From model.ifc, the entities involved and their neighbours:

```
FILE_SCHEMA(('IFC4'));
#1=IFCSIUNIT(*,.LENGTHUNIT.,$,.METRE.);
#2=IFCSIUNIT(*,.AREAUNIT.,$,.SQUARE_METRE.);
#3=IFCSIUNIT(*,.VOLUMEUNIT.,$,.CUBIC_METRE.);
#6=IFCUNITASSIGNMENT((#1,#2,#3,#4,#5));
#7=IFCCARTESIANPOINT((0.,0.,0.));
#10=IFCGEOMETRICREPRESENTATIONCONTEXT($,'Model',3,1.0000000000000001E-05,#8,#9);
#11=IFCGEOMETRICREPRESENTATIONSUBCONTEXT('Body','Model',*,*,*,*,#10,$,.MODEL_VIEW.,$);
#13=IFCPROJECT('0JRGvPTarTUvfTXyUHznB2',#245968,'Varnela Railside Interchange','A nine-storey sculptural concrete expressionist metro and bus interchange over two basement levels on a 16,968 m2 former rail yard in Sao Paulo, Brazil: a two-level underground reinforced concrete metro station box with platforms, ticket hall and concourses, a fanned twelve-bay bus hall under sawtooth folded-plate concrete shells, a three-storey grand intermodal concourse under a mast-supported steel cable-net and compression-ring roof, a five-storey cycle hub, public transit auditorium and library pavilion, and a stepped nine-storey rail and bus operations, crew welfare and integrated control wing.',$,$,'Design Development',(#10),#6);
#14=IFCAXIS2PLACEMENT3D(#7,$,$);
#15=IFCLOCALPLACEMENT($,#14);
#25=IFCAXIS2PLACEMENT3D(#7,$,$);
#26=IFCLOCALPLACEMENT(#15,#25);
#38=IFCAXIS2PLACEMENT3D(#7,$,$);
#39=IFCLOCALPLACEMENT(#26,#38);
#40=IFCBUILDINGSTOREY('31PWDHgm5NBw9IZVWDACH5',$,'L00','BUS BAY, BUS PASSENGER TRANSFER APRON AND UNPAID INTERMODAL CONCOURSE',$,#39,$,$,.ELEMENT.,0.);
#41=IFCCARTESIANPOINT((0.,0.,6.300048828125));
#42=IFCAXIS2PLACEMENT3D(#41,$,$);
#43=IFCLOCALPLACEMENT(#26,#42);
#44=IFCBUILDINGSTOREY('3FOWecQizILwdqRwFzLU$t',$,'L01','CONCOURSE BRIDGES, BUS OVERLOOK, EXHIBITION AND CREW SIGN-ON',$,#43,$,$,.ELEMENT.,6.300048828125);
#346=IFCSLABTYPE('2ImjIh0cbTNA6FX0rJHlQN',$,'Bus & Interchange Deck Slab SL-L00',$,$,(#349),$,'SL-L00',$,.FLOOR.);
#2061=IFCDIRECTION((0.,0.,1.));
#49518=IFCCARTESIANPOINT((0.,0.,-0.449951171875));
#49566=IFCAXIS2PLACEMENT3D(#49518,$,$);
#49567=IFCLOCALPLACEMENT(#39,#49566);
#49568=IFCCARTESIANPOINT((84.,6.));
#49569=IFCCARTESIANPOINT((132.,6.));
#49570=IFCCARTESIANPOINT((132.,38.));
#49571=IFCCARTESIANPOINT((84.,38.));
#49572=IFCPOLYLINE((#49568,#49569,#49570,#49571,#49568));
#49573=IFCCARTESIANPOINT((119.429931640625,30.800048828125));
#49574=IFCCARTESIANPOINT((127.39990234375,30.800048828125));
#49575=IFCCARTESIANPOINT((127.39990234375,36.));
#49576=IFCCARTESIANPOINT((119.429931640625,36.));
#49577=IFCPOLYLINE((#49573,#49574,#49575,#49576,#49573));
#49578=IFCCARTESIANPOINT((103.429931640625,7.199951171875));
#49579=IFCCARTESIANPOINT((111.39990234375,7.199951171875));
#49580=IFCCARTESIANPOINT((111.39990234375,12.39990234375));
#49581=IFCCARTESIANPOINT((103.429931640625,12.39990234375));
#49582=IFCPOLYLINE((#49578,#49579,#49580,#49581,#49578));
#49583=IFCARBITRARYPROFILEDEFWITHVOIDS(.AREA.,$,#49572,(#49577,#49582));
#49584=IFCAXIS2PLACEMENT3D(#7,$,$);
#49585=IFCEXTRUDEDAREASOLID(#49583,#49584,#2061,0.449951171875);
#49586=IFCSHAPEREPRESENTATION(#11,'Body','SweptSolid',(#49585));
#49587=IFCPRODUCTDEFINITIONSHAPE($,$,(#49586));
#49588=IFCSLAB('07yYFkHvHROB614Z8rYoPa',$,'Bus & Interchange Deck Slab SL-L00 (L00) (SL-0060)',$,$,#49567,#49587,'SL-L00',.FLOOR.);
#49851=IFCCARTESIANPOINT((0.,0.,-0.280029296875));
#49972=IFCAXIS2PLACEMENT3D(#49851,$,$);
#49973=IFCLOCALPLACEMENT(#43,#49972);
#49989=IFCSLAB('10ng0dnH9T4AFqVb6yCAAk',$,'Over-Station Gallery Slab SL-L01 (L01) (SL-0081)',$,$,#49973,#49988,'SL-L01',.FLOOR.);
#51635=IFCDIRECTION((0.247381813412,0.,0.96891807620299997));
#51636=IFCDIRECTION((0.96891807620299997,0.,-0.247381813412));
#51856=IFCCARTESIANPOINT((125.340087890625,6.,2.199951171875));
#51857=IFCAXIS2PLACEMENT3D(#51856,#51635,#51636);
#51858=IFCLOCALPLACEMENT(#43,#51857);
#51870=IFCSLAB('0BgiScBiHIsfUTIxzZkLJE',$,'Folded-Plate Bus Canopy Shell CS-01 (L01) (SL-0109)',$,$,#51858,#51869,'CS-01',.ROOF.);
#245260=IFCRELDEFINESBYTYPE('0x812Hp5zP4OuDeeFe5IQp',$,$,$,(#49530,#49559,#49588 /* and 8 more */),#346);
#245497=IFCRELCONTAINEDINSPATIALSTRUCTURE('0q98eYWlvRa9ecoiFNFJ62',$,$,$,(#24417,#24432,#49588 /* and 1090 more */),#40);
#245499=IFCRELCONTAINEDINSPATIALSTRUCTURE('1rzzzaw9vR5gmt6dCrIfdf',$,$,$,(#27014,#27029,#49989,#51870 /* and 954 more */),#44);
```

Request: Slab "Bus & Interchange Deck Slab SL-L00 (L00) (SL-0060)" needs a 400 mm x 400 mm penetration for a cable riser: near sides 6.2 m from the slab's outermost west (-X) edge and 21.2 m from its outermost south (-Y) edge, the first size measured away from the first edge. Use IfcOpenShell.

```python
import numpy as np
import ifcopenshell
import ifcopenshell.api.feature
import ifcopenshell.api.geometry
import ifcopenshell.api.root
import ifcopenshell.geom
import ifcopenshell.util.placement
import ifcopenshell.util.representation
import ifcopenshell.util.shape
import ifcopenshell.util.unit

model = ifcopenshell.open("model.ifc")
unit_scale = ifcopenshell.util.unit.calculate_unit_scale(model)
settings = ifcopenshell.geom.settings()


def volume(element):
    """Net volume in cubic metres, openings subtracted."""
    shape = ifcopenshell.geom.create_shape(settings, element)
    return ifcopenshell.util.shape.get_volume(shape.geometry)


slab = model.by_guid("07yYFkHvHROB614Z8rYoPa")
before = volume(slab)

# Extent in the slab's own axes, in metres. The edges named are its -X and -Y sides.
slab_shape = ifcopenshell.geom.create_shape(settings, slab)
vertices = ifcopenshell.util.shape.get_vertices(slab_shape.geometry)
x_min, y_min, bottom = vertices.min(axis=0)
top = vertices[:, 2].max()

opening = ifcopenshell.api.root.create_entity(model, ifc_class="IfcOpeningElement", name="Cable riser opening", predefined_type="OPENING")
context = ifcopenshell.util.representation.get_context(model, "Model", "Body", "MODEL_VIEW")
width, depth = 0.4, 0.4
outline = [(0.0, 0.0), (width, 0.0), (width, depth), (0.0, depth), (0.0, 0.0)]
# Overshoot both faces by 50 mm so the cut is clean.
shape = ifcopenshell.api.geometry.add_slab_representation(
    model, context=context, depth=top - bottom + 0.1, polyline=outline
)
ifcopenshell.api.geometry.assign_representation(model, product=opening, representation=shape)

matrix = ifcopenshell.util.placement.get_local_placement(slab.ObjectPlacement)
matrix[:, 3] = matrix @ np.append(np.array([x_min + 6.2, y_min + 21.2, bottom - 0.05]) / unit_scale, 1.0)
ifcopenshell.api.geometry.edit_object_placement(model, product=opening, matrix=matrix, is_si=False)
ifcopenshell.api.feature.add_feature(model, feature=opening, element=slab)

after = volume(slab)

print(f"slab volume {before:.3f} -> {after:.3f} m3")

model.write("model_v2.ifc")
```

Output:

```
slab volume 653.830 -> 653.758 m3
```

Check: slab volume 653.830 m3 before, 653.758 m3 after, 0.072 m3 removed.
